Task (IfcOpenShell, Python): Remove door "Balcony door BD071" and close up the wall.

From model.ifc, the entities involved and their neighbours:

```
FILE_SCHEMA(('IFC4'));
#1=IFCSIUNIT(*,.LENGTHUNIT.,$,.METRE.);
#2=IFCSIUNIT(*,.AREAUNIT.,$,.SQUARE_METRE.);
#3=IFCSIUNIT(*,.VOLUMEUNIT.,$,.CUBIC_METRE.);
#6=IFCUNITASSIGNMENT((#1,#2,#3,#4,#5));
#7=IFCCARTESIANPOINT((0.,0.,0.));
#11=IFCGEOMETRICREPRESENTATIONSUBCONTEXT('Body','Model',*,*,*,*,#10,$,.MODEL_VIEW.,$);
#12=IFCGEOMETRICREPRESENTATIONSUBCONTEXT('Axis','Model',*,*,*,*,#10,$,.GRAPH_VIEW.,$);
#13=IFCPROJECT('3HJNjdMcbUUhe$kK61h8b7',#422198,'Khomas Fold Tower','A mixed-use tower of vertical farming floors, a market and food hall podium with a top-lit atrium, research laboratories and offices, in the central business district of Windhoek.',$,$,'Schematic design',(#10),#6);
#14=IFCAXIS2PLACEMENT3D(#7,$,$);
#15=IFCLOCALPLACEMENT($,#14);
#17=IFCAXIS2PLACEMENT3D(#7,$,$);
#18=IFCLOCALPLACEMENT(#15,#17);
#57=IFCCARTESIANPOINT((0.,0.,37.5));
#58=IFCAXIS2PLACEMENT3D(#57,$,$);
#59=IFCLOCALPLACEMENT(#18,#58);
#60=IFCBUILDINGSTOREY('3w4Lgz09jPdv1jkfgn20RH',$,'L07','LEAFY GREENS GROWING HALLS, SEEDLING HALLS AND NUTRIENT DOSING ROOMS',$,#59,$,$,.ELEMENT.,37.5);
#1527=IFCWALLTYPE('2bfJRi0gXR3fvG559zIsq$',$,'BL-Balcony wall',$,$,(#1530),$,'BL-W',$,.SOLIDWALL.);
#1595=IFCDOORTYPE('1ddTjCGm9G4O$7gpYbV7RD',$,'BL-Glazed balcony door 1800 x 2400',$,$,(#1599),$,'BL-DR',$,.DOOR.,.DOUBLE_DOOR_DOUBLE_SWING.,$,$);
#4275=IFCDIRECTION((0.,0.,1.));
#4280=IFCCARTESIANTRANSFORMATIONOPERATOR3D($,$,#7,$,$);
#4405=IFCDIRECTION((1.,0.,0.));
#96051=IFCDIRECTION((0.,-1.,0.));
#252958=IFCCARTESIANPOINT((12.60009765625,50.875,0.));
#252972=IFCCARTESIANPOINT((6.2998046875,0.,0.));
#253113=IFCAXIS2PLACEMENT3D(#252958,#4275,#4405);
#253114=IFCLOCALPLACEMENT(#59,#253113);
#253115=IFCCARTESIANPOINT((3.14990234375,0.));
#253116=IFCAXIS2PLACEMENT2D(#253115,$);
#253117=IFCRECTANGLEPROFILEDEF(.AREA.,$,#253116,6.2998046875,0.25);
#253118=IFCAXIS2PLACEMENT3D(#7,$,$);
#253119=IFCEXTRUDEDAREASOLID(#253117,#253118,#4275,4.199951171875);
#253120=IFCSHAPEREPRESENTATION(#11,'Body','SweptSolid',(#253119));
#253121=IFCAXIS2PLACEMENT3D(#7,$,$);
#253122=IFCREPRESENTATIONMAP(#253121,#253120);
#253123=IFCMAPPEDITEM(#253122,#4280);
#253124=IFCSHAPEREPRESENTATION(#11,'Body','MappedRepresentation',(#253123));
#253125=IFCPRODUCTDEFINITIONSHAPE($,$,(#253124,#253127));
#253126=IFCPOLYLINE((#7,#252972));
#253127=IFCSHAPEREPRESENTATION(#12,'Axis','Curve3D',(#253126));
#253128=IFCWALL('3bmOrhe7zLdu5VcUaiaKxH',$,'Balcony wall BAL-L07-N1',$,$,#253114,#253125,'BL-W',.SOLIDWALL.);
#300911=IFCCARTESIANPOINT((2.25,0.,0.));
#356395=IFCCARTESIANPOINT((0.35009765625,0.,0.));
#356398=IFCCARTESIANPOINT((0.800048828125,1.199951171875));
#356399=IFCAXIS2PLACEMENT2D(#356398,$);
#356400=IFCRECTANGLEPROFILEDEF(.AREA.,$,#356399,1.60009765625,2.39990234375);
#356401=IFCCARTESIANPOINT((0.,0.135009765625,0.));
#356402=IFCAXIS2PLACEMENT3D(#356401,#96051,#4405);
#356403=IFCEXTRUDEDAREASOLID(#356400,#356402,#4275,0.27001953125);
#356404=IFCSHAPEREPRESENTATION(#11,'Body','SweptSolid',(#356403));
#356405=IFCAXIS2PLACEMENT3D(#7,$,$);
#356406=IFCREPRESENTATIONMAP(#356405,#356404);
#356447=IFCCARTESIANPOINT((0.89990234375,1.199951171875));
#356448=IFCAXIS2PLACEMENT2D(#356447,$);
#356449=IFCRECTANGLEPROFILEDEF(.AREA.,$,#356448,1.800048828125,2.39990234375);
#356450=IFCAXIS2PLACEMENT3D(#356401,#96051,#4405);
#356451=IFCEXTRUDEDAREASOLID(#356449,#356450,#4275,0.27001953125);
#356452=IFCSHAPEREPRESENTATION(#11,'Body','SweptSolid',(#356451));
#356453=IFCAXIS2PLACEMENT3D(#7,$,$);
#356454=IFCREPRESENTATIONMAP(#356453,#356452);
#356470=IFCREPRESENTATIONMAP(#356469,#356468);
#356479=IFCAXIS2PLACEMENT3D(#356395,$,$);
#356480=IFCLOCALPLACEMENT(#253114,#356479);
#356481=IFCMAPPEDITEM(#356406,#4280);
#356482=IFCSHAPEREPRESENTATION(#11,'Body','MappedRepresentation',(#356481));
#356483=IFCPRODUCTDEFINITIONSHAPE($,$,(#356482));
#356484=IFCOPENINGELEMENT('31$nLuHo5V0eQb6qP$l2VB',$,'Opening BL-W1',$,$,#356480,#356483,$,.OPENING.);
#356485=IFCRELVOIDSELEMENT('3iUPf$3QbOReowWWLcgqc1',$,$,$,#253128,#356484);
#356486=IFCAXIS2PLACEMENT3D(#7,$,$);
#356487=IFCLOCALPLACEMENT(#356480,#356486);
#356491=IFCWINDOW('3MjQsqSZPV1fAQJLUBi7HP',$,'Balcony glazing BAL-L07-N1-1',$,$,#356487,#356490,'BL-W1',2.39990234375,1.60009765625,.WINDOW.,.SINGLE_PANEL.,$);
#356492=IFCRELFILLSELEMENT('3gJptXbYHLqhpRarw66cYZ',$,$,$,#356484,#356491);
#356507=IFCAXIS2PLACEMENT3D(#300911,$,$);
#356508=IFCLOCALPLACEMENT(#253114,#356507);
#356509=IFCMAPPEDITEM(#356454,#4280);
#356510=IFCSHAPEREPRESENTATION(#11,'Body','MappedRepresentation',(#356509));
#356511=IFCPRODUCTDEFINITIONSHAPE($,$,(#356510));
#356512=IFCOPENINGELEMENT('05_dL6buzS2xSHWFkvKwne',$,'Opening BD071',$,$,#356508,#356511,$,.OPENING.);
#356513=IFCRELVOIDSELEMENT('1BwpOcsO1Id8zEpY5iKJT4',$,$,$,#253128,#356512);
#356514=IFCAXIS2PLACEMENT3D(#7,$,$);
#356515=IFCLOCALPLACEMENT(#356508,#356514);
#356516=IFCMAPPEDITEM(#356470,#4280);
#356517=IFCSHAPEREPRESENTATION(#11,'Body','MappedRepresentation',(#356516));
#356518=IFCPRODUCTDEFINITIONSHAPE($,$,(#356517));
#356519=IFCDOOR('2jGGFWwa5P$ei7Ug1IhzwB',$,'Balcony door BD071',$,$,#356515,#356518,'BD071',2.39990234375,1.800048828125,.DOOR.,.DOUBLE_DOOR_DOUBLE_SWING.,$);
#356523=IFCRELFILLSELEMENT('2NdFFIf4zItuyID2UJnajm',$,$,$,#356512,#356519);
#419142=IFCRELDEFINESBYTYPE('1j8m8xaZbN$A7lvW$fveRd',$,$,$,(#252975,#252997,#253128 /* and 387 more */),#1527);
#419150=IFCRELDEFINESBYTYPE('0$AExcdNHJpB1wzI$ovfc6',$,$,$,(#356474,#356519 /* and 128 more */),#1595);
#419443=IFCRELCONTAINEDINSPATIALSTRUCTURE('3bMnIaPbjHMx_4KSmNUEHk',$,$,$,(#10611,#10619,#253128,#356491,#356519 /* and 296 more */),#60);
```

```python
import ifcopenshell
import ifcopenshell.api.feature
import ifcopenshell.api.root
import ifcopenshell.geom
import ifcopenshell.util.shape

model = ifcopenshell.open("model.ifc")
settings = ifcopenshell.geom.settings()


def volume(element):
    """Net volume in cubic metres, openings subtracted."""
    shape = ifcopenshell.geom.create_shape(settings, element)
    return ifcopenshell.util.shape.get_volume(shape.geometry)


door = model.by_guid("2jGGFWwa5P$ei7Ug1IhzwB")
opening = door.FillsVoids[0].RelatingOpeningElement
wall = opening.VoidsElements[0].RelatingBuildingElement
before = volume(wall)

ifcopenshell.api.root.remove_product(model, product=door)
ifcopenshell.api.feature.remove_feature(model, feature=opening)

after = volume(wall)

print(f"wall volume {before:.3f} -> {after:.3f} m3")

model.write("model_updated.ifc")
```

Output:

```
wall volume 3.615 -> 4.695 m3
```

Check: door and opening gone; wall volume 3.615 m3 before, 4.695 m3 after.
